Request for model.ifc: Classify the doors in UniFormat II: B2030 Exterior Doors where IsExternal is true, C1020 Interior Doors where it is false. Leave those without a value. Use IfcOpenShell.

First a look at what the model holds.

```python
import ifcopenshell
import ifcopenshell.util.element

model = ifcopenshell.open("model.ifc")
print(model.schema)
print("classifications:", [c.Name for c in model.by_type("IfcClassification")])
values = [ifcopenshell.util.element.get_pset(e, "Pset_DoorCommon", "IsExternal") for e in model.by_type("IfcDoor")]
for value in (True, False, None):
    print("IsExternal", value, values.count(value))
```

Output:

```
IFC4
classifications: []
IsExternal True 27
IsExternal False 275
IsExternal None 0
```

```python
import ifcopenshell
import ifcopenshell.api.classification
import ifcopenshell.util.element

model = ifcopenshell.open("model.ifc")

system = ifcopenshell.api.classification.add_classification(model, classification="UniFormat II")

doors = model.by_type("IfcDoor")
external = {e: ifcopenshell.util.element.get_pset(e, "Pset_DoorCommon", "IsExternal") for e in doors}
for flag, code, name in ((True, "B2030", "Exterior Doors"), (False, "C1020", "Interior Doors")):
    products = [e for e in doors if external[e] is flag]
    ifcopenshell.api.classification.add_reference(
        model, products=products, classification=system, identification=code, name=name
    )
    print(code, len(products))

model.write("model_rev.ifc")
```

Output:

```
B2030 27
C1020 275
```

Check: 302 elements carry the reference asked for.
